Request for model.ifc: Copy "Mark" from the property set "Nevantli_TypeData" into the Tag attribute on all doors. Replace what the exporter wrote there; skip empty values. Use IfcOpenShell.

First a look at what the model holds.

```python
import ifcopenshell
import ifcopenshell.util.element

model = ifcopenshell.open("model.ifc")
print(model.schema)
doors = model.by_type("IfcDoor")
print(len(doors), "doors")
for e in doors[:8]:
    source = ifcopenshell.util.element.get_pset(e, "Nevantli_TypeData", "Mark")
    target = e.Tag
    print(e.id(), repr(source), repr(target), sep=" | ")
```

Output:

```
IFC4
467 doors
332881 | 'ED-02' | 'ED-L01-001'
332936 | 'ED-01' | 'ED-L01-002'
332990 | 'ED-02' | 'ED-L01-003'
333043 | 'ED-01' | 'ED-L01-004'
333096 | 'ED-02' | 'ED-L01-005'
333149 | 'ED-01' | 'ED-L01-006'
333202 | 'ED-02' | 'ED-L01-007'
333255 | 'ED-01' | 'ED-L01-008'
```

```python
import ifcopenshell
import ifcopenshell.util.element

model = ifcopenshell.open("model.ifc")

count = 0
for e in model.by_type("IfcDoor"):
    value = ifcopenshell.util.element.get_pset(e, "Nevantli_TypeData", "Mark")
    current = e.Tag
    if not value or not value.strip() or current == value:
        continue
    e.Tag = value
    count += 1

print(count, "doors updated")

model.write("model_updated.ifc")
```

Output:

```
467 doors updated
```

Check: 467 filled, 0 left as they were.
